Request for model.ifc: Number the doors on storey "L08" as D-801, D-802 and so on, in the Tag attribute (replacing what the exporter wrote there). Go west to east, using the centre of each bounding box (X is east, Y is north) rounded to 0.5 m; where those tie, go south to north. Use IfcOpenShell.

First a look at what the model holds.

```python
import ifcopenshell
import ifcopenshell.util.element
import ifcopenshell.util.placement

model = ifcopenshell.open("model.ifc")
print(model.schema)
storey = next(s for s in model.by_type("IfcBuildingStorey") if s.Name == "L08")
doors = [e for e in ifcopenshell.util.element.get_decomposition(storey) if e.is_a("IfcDoor")]
for e in sorted(doors, key=lambda e: e.id()):
    origin = ifcopenshell.util.placement.get_local_placement(e.ObjectPlacement)[:3, 3]
    print(e.id(), e.Tag, e.Name, origin.round(2) + 0.0, sep=" | ")
```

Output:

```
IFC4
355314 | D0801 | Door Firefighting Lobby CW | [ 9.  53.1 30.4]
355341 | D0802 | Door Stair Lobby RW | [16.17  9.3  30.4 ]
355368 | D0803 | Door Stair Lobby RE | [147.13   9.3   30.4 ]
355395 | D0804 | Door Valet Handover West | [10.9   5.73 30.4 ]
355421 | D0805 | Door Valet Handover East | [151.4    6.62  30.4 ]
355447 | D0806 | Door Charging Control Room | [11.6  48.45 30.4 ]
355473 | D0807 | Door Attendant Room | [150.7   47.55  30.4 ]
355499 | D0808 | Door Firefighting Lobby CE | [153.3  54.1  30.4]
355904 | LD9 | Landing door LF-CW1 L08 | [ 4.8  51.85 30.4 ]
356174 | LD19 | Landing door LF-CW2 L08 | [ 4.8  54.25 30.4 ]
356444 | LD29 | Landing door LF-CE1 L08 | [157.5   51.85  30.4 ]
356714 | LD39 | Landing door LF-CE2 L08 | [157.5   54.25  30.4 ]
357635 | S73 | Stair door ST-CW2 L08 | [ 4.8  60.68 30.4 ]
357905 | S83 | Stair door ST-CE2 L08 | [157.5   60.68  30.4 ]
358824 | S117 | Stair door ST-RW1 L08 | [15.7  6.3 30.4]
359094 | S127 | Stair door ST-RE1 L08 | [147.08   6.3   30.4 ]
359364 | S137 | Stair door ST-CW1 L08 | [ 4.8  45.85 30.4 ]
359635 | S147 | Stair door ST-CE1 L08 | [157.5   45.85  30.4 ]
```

```python
import ifcopenshell
import ifcopenshell.geom
import ifcopenshell.util.element
import ifcopenshell.util.shape

model = ifcopenshell.open("model.ifc")
settings = ifcopenshell.geom.settings()
settings.set("use-world-coords", True)


def centre(element):
    shape = ifcopenshell.geom.create_shape(settings, element)
    return ifcopenshell.util.shape.get_bbox_centroid(shape.geometry)


storey = next(s for s in model.by_type("IfcBuildingStorey") if s.Name == "L08")
doors = [e for e in ifcopenshell.util.element.get_decomposition(storey) if e.is_a("IfcDoor")]

# Insertion points can sit at a corner or the storey origin, so sort by the geometry (in metres).
centres = {e: centre(e) for e in doors}
doors.sort(key=lambda e: (round(centres[e][0] / 0.5), centres[e][1]))

for i, e in enumerate(doors, start=1):
    number = f"D-8{i:02d}"
    e.Tag = number
    print(e.id(), number)

model.write("model_edited.ifc")
```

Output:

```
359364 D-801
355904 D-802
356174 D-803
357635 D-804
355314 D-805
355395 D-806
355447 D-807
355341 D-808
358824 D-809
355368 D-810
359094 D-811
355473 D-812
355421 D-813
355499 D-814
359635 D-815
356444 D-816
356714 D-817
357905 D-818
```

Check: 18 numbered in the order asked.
